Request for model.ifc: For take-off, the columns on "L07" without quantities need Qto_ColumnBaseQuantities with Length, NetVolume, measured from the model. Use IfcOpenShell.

First a look at what the model holds.

```python
import ifcopenshell
import ifcopenshell.util.element
import ifcopenshell.util.unit

model = ifcopenshell.open("model.ifc")
print(model.schema)
for unit_type in ("LENGTHUNIT", "AREAUNIT", "VOLUMEUNIT"):
    print(unit_type, ifcopenshell.util.unit.calculate_unit_scale(model, unit_type))
storey = next(s for s in model.by_type("IfcBuildingStorey") if s.Name == "L07")
columns = [e for e in ifcopenshell.util.element.get_decomposition(storey) if e.is_a("IfcColumn")]
for e in sorted(columns, key=lambda e: e.id()):
    print(e.id(), e.is_a(), e.Name, list(ifcopenshell.util.element.get_psets(e, qtos_only=True)), sep=" | ")
```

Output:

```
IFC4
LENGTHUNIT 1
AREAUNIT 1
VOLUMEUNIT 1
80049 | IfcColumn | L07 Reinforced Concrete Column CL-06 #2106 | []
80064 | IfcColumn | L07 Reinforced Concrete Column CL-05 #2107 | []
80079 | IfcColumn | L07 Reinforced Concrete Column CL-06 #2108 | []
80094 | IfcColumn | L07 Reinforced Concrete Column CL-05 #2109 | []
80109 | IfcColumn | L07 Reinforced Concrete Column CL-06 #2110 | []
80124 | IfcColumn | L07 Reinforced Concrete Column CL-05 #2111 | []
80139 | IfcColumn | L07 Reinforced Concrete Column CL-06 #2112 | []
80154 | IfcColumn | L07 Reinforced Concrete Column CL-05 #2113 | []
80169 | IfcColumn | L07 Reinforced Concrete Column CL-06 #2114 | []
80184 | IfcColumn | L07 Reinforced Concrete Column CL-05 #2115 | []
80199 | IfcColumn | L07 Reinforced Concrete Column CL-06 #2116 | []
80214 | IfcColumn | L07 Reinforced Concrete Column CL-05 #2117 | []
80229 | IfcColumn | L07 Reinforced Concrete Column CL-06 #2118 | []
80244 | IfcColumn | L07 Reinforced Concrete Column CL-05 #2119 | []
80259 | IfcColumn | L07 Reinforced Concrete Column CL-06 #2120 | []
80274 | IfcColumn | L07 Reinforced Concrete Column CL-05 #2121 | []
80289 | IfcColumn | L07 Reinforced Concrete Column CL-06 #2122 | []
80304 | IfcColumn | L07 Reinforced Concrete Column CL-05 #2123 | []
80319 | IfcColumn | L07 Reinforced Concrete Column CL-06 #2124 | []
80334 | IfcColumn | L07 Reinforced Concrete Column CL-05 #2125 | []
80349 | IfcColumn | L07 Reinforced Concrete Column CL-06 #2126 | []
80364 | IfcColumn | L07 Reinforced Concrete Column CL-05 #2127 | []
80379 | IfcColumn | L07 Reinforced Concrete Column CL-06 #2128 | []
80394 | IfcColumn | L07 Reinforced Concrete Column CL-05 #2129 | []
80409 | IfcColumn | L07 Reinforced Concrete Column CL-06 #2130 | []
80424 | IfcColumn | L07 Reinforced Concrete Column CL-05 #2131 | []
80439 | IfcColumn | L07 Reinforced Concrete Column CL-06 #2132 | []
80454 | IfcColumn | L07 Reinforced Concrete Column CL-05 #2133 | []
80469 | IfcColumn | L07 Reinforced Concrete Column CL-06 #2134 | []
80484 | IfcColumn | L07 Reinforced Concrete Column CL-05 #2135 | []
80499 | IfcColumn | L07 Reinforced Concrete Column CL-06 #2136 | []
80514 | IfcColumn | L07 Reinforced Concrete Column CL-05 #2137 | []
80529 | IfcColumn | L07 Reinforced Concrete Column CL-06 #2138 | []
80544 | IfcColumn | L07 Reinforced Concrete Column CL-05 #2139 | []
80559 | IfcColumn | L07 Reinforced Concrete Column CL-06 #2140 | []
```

```python
import ifcopenshell
import ifcopenshell.api.pset
import ifcopenshell.geom
import ifcopenshell.util.element
import ifcopenshell.util.shape
import ifcopenshell.util.unit

model = ifcopenshell.open("model.ifc")
unit_scale = ifcopenshell.util.unit.calculate_unit_scale(model)
volume_scale = ifcopenshell.util.unit.calculate_unit_scale(model, "VOLUMEUNIT")
settings = ifcopenshell.geom.settings()

storey = next(s for s in model.by_type("IfcBuildingStorey") if s.Name == "L07")
columns = [e for e in ifcopenshell.util.element.get_decomposition(storey) if e.is_a("IfcColumn")]

for e in sorted(columns, key=lambda e: e.id()):
    if ifcopenshell.util.element.get_psets(e, qtos_only=True, should_inherit=False):
        continue
    # Geometry comes back in metres, in the element's own axes.
    shape = ifcopenshell.geom.create_shape(settings, e)
    values = {
        "Length": ifcopenshell.util.shape.get_z(shape.geometry) / unit_scale,
        "NetVolume": ifcopenshell.util.shape.get_volume(shape.geometry) / volume_scale,
    }
    qto = ifcopenshell.api.pset.add_qto(model, product=e, name="Qto_ColumnBaseQuantities")
    ifcopenshell.api.pset.edit_qto(model, qto=qto, properties=values)
    print(e.id(), {k: round(v, 3) for k, v in values.items()})

model.write("model_edited.ifc")
```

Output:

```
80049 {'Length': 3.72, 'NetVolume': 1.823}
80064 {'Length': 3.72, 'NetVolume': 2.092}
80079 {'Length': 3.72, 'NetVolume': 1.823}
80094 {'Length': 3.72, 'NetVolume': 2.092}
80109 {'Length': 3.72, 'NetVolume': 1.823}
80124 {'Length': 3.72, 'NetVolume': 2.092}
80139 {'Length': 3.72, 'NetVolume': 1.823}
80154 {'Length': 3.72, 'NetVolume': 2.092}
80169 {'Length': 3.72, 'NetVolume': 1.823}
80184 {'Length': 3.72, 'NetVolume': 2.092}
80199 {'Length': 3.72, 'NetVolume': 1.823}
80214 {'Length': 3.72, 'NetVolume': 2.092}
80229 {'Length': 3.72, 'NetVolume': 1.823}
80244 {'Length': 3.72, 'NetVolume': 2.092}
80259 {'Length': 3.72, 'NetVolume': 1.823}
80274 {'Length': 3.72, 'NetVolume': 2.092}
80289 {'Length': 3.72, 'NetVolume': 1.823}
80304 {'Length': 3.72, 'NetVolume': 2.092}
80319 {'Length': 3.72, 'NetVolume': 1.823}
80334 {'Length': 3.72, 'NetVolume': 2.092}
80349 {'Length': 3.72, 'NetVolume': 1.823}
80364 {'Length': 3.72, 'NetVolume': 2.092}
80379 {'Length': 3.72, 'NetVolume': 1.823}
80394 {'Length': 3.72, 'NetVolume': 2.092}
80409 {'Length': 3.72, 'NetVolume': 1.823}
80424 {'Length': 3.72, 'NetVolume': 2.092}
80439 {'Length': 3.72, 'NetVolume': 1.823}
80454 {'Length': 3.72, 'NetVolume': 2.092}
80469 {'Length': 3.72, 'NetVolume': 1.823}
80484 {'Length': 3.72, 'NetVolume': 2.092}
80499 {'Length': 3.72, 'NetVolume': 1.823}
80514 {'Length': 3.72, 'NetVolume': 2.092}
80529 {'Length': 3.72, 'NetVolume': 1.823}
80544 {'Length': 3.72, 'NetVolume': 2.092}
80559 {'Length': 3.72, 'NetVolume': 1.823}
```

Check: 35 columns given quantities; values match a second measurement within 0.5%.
